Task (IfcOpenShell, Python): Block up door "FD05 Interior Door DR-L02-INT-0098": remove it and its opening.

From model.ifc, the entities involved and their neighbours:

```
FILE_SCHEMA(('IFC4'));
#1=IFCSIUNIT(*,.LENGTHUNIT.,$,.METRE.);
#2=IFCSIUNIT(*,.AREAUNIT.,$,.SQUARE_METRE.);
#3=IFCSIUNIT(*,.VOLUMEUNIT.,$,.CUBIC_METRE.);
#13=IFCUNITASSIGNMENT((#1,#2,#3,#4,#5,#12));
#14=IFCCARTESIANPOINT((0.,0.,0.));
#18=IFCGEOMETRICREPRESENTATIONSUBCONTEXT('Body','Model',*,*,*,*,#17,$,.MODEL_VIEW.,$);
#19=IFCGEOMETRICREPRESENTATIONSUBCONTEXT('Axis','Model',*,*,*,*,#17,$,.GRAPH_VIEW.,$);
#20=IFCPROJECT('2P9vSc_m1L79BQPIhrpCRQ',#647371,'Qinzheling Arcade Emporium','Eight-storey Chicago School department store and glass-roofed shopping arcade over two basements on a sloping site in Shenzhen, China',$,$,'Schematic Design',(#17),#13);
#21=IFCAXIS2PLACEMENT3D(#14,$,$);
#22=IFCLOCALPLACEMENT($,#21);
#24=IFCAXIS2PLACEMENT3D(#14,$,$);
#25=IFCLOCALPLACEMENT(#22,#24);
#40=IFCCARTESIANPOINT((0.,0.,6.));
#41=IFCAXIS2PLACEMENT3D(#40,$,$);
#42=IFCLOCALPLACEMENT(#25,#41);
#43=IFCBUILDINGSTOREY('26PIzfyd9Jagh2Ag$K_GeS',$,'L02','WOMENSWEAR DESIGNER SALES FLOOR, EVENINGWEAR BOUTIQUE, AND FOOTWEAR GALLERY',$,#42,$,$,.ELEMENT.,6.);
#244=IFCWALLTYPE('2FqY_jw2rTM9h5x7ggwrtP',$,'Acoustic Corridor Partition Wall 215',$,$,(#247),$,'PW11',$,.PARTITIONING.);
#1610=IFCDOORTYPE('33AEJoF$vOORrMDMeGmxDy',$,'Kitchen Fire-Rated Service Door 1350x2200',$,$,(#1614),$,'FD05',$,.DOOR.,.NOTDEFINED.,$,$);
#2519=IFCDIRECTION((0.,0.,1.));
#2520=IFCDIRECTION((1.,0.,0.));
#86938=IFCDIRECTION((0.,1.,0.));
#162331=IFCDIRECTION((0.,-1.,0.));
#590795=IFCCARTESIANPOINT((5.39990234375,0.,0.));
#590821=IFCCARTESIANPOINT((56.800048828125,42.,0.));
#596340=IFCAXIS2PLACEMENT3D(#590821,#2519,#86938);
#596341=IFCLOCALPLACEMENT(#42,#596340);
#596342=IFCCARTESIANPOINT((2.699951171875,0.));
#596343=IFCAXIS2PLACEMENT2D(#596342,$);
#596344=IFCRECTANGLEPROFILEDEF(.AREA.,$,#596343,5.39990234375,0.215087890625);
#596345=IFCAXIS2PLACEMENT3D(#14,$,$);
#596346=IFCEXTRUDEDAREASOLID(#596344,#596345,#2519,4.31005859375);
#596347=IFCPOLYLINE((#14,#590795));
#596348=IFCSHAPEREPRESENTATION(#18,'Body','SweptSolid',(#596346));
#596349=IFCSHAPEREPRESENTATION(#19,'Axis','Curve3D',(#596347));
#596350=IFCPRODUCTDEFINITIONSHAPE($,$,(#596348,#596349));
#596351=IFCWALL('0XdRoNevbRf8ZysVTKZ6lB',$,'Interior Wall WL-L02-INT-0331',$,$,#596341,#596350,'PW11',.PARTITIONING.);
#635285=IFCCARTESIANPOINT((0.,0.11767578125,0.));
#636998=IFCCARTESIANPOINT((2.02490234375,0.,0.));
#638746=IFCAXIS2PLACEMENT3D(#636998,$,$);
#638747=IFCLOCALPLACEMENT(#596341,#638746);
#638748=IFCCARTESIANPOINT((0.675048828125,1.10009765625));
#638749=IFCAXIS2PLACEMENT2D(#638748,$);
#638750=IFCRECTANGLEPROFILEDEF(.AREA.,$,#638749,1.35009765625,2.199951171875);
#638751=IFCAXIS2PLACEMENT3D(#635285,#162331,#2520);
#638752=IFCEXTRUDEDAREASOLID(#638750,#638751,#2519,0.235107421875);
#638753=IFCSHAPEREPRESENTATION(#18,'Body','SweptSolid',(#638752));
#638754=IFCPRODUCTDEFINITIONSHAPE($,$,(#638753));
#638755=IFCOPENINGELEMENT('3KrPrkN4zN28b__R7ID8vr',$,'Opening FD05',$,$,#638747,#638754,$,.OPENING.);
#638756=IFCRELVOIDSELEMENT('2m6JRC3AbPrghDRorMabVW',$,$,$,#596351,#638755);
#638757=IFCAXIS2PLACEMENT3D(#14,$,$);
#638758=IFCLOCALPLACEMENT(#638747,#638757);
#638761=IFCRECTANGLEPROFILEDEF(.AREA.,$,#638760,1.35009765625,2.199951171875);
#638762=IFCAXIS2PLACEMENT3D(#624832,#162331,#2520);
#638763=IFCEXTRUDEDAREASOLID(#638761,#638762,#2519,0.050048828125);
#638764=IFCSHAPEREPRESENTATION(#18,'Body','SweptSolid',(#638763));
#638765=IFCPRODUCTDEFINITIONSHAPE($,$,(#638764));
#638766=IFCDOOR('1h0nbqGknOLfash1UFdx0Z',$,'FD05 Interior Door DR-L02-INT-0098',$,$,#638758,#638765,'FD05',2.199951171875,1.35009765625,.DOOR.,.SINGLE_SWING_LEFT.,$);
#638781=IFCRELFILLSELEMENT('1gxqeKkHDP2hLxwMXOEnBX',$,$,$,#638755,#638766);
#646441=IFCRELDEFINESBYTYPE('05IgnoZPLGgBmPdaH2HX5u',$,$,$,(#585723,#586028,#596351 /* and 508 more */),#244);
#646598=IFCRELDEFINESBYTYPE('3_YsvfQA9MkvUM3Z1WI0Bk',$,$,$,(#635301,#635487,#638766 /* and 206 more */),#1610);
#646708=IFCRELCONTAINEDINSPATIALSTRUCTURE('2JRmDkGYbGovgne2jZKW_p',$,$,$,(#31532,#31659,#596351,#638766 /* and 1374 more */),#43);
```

```python
import ifcopenshell
import ifcopenshell.api.feature
import ifcopenshell.api.root
import ifcopenshell.geom
import ifcopenshell.util.shape

model = ifcopenshell.open("model.ifc")
settings = ifcopenshell.geom.settings()


def volume(element):
    """Net volume in cubic metres, openings subtracted."""
    shape = ifcopenshell.geom.create_shape(settings, element)
    return ifcopenshell.util.shape.get_volume(shape.geometry)


door = model.by_guid("1h0nbqGknOLfash1UFdx0Z")
opening = door.FillsVoids[0].RelatingOpeningElement
wall = opening.VoidsElements[0].RelatingBuildingElement
before = volume(wall)

ifcopenshell.api.root.remove_product(model, product=door)
ifcopenshell.api.feature.remove_feature(model, feature=opening)

after = volume(wall)

print(f"wall volume {before:.3f} -> {after:.3f} m3")

model.write("model-out.ifc")
```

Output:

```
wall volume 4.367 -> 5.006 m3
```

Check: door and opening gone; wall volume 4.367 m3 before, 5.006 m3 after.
